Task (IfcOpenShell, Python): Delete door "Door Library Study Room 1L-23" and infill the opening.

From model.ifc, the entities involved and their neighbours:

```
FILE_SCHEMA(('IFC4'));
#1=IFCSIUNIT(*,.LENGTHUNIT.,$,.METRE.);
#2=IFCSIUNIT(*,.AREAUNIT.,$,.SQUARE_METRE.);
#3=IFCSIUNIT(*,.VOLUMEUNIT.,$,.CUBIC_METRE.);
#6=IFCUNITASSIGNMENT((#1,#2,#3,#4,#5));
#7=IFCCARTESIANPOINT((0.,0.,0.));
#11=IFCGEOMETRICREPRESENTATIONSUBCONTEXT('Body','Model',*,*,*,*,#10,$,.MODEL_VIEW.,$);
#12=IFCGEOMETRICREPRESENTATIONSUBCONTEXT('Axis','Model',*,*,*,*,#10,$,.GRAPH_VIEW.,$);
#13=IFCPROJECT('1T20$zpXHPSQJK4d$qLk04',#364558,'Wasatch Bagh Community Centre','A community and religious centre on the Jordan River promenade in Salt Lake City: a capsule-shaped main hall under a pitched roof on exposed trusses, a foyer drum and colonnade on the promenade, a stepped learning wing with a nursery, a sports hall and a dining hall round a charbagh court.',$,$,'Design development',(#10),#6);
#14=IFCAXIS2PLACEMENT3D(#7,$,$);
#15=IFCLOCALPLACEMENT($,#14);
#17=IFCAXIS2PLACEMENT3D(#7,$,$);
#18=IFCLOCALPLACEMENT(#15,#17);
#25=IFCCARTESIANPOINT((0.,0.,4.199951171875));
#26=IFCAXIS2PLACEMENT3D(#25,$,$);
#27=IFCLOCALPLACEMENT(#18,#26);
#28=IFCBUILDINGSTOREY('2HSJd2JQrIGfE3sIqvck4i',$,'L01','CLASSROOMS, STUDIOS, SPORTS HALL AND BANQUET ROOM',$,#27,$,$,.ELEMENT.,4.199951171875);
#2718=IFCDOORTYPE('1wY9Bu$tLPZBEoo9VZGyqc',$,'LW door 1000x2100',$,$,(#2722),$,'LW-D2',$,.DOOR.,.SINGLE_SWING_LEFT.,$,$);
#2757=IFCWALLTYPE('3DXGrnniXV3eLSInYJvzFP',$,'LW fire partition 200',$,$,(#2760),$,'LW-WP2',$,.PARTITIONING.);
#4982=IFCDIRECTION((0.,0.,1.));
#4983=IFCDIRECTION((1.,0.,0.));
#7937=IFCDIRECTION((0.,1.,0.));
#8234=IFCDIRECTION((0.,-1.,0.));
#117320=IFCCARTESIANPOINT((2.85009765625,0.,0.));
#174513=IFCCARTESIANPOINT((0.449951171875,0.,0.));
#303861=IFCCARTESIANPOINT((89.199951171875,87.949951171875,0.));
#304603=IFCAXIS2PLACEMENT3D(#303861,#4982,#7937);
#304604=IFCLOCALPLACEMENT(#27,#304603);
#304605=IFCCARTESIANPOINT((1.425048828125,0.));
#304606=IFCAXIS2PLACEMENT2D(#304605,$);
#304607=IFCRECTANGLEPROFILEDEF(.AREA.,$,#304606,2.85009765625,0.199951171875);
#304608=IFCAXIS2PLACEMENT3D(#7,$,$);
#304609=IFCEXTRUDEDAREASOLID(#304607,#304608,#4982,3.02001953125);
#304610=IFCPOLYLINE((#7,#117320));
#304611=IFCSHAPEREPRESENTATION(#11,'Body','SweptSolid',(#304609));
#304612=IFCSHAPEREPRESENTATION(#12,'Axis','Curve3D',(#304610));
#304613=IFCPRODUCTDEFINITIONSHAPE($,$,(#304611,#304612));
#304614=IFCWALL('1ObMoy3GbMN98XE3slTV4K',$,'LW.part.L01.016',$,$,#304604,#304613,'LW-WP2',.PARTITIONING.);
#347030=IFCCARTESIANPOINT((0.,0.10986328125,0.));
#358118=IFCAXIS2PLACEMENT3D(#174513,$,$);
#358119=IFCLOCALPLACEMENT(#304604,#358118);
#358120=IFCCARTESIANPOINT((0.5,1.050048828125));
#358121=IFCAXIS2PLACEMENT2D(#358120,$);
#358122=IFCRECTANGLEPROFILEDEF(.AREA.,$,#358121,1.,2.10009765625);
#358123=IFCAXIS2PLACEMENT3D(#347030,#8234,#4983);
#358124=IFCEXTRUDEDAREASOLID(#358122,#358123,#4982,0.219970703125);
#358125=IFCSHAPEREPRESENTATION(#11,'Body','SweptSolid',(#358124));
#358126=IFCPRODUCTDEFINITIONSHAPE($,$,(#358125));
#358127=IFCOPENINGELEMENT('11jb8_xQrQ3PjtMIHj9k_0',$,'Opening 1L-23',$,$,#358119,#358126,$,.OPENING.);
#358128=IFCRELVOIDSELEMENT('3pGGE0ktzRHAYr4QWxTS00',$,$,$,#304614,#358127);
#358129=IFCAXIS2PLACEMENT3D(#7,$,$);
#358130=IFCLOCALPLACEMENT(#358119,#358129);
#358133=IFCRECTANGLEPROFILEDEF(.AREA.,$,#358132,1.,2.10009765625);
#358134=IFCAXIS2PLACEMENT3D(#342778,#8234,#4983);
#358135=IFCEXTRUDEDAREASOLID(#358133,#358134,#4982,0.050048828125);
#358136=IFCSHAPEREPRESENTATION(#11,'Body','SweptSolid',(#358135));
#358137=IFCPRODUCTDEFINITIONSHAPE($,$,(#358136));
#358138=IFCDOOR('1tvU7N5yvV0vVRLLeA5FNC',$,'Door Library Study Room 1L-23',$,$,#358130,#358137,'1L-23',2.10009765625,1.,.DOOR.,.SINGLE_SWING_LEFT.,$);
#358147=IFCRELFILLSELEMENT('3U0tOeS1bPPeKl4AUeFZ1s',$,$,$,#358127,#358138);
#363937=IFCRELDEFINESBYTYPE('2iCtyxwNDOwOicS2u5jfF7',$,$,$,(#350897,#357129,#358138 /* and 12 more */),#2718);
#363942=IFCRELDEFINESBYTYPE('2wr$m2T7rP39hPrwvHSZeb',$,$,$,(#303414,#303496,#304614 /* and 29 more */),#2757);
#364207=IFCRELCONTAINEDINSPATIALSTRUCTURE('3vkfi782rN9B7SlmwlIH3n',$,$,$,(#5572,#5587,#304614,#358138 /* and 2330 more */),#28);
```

```python
import ifcopenshell
import ifcopenshell.api.feature
import ifcopenshell.api.root
import ifcopenshell.geom
import ifcopenshell.util.shape

model = ifcopenshell.open("model.ifc")
settings = ifcopenshell.geom.settings()


def volume(element):
    """Net volume in cubic metres, openings subtracted."""
    shape = ifcopenshell.geom.create_shape(settings, element)
    return ifcopenshell.util.shape.get_volume(shape.geometry)


door = model.by_id(358138)
opening = door.FillsVoids[0].RelatingOpeningElement
wall = opening.VoidsElements[0].RelatingBuildingElement
before = volume(wall)

ifcopenshell.api.root.remove_product(model, product=door)
ifcopenshell.api.feature.remove_feature(model, feature=opening)

after = volume(wall)

print(f"wall volume {before:.3f} -> {after:.3f} m3")

model.write("model_updated.ifc")
```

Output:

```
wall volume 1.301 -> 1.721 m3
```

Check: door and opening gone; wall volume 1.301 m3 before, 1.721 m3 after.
